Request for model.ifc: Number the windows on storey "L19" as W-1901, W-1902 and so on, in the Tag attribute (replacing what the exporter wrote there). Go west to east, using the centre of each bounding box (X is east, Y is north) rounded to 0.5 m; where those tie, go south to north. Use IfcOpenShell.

First a look at what the model holds.

```python
import ifcopenshell
import ifcopenshell.util.element
import ifcopenshell.util.placement

model = ifcopenshell.open("model.ifc")
print(model.schema)
storey = next(s for s in model.by_type("IfcBuildingStorey") if s.Name == "L19")
windows = [e for e in ifcopenshell.util.element.get_decomposition(storey) if e.is_a("IfcWindow")]
for e in sorted(windows, key=lambda e: e.id()):
    origin = ifcopenshell.util.placement.get_local_placement(e.ObjectPlacement)[:3, 3]
    print(e.id(), e.Tag, e.Name, origin.round(2) + 0.0, sep=" | ")
```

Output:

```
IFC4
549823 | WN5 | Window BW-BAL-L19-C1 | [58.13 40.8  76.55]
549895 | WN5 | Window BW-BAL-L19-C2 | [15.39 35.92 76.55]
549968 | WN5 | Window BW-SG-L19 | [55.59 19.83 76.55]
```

```python
import ifcopenshell
import ifcopenshell.geom
import ifcopenshell.util.element
import ifcopenshell.util.shape

model = ifcopenshell.open("model.ifc")
settings = ifcopenshell.geom.settings()
settings.set("use-world-coords", True)


def centre(element):
    shape = ifcopenshell.geom.create_shape(settings, element)
    return ifcopenshell.util.shape.get_bbox_centroid(shape.geometry)


storey = next(s for s in model.by_type("IfcBuildingStorey") if s.Name == "L19")
windows = [e for e in ifcopenshell.util.element.get_decomposition(storey) if e.is_a("IfcWindow")]

# Insertion points can sit at a corner or the storey origin, so sort by the geometry (in metres).
centres = {e: centre(e) for e in windows}
windows.sort(key=lambda e: (round(centres[e][0] / 0.5), centres[e][1]))

for i, e in enumerate(windows, start=1):
    number = f"W-19{i:02d}"
    e.Tag = number
    print(e.id(), number)

model.write("model_rev.ifc")
```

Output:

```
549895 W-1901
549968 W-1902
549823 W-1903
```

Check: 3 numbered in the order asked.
